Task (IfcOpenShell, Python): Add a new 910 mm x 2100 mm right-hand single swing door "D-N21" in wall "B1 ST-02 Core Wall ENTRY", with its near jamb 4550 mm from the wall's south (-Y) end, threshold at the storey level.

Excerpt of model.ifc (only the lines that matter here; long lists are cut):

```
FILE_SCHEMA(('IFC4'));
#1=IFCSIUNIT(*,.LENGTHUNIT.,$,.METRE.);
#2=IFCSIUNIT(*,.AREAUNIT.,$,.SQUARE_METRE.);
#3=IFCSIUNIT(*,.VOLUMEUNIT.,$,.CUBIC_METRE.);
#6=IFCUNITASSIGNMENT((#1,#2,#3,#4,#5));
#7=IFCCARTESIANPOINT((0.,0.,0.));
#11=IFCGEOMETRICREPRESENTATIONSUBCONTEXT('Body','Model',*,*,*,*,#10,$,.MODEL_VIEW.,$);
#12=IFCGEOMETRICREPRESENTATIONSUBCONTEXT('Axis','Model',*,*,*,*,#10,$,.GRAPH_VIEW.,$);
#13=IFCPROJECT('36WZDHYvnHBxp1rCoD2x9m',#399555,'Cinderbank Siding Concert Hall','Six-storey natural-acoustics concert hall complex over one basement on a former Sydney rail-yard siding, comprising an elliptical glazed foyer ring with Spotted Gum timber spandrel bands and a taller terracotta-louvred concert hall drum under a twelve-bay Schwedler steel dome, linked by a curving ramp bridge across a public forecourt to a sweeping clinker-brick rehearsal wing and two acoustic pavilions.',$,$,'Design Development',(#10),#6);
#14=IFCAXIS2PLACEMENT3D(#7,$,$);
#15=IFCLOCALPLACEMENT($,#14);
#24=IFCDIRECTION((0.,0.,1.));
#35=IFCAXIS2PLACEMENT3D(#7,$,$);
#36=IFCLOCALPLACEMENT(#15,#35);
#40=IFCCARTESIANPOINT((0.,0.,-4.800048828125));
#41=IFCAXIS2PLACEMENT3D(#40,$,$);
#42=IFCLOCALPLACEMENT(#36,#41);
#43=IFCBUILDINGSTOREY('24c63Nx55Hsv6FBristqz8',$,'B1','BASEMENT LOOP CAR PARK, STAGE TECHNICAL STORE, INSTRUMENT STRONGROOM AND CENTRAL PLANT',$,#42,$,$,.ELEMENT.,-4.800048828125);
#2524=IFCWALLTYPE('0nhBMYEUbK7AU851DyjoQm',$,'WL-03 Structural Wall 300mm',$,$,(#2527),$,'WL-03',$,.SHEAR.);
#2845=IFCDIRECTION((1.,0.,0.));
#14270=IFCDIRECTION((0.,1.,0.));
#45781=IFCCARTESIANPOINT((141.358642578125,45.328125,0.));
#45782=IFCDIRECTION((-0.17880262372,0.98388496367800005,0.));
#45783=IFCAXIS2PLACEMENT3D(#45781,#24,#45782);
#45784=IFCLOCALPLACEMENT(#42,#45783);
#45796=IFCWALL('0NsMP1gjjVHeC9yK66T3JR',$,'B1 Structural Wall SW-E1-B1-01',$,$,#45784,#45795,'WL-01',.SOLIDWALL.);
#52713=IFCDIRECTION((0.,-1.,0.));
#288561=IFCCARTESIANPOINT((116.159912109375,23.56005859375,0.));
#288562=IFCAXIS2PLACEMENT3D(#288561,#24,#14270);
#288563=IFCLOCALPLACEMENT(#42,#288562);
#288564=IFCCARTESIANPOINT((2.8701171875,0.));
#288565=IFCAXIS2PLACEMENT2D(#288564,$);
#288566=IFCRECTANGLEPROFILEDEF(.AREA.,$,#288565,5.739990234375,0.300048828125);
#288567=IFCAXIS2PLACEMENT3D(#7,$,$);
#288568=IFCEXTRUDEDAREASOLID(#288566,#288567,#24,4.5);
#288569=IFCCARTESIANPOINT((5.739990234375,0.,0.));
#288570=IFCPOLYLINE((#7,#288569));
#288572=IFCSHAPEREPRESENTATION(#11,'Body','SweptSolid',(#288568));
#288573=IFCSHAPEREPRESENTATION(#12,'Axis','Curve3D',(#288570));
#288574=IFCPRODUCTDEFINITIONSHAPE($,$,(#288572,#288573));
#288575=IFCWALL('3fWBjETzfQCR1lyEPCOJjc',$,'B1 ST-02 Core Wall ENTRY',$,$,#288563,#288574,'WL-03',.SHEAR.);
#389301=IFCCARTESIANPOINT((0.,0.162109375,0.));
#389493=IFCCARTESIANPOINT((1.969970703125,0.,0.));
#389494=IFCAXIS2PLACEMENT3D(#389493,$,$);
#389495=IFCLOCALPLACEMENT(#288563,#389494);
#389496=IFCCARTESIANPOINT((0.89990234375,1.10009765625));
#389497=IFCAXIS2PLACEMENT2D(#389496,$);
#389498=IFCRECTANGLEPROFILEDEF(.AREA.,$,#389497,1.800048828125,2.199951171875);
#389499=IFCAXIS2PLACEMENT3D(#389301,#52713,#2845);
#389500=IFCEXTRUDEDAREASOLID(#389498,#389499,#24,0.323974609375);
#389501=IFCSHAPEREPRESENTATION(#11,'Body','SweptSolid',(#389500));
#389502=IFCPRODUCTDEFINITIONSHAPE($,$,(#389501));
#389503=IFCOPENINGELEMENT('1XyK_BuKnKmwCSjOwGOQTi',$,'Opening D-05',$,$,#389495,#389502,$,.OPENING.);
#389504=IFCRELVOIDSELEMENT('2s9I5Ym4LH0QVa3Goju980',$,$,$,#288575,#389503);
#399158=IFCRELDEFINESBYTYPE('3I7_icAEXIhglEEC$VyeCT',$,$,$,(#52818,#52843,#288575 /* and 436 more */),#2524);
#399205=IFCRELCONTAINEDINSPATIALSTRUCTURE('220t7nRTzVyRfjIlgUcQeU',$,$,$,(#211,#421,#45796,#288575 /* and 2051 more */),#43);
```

```python
import numpy as np
import ifcopenshell
import ifcopenshell.api.feature
import ifcopenshell.api.geometry
import ifcopenshell.api.root
import ifcopenshell.api.spatial
import ifcopenshell.geom
import ifcopenshell.util.element
import ifcopenshell.util.placement
import ifcopenshell.util.representation
import ifcopenshell.util.shape
import ifcopenshell.util.unit

model = ifcopenshell.open("model.ifc")
unit_scale = ifcopenshell.util.unit.calculate_unit_scale(model)
settings = ifcopenshell.geom.settings()


def volume(element):
    """Net volume in cubic metres, openings subtracted."""
    shape = ifcopenshell.geom.create_shape(settings, element)
    return ifcopenshell.util.shape.get_volume(shape.geometry)


wall = model.by_guid("3fWBjETzfQCR1lyEPCOJjc")
storey = ifcopenshell.util.element.get_container(wall, ifc_class="IfcBuildingStorey")
context = ifcopenshell.util.representation.get_context(model, "Model", "Body", "MODEL_VIEW")
before = volume(wall)

width, height, from_end, sill = 0.91, 2.1, 4.55, 0.0  # metres

# The wall runs along its own X axis, and the end named is its -X end.
wall_shape = ifcopenshell.geom.create_shape(settings, wall)
x, y, z = ifcopenshell.util.shape.get_vertices(wall_shape.geometry).T
start = x.min() + from_end
face, thickness = float(y.min()), float(y.max() - y.min())
wall_matrix = ifcopenshell.util.placement.get_local_placement(wall.ObjectPlacement)
level = ifcopenshell.util.placement.get_local_placement(storey.ObjectPlacement)[2, 3]


def in_wall(x, y):
    """Placement at x, y metres in the wall's axes, at sill height."""
    matrix = wall_matrix.copy()
    matrix[:, 3] = wall_matrix @ np.array([x / unit_scale, y / unit_scale, 0.0, 1.0])
    matrix[2, 3] = level + sill / unit_scale
    return matrix


# Opening: a box that overshoots both wall faces by 50 mm.
opening = ifcopenshell.api.root.create_entity(model, ifc_class="IfcOpeningElement", predefined_type="OPENING")
box = ifcopenshell.api.geometry.add_wall_representation(
    model, context=context, length=width, height=height, thickness=thickness + 0.1
)
ifcopenshell.api.geometry.assign_representation(model, product=opening, representation=box)
ifcopenshell.api.geometry.edit_object_placement(model, product=opening, matrix=in_wall(start, face - 0.05), is_si=False)
ifcopenshell.api.feature.add_feature(model, feature=opening, element=wall)

door = ifcopenshell.api.root.create_entity(model, ifc_class="IfcDoor", name="D-N21", predefined_type="DOOR")
door.OverallWidth, door.OverallHeight = width / unit_scale, height / unit_scale
door.OperationType = "SINGLE_SWING_RIGHT"
body = ifcopenshell.api.geometry.add_door_representation(
    model,
    context=context,
    overall_width=door.OverallWidth,
    overall_height=door.OverallHeight,
    operation_type="SINGLE_SWING_RIGHT",
    lining_properties={"LiningDepth": thickness / unit_scale, "ThresholdDepth": thickness / unit_scale},
)
ifcopenshell.api.geometry.assign_representation(model, product=door, representation=body)
ifcopenshell.api.spatial.assign_container(model, products=[door], relating_structure=storey)
ifcopenshell.api.feature.add_filling(model, opening=opening, element=door)

# The lining spans the wall, so the door starts at the wall face.
ifcopenshell.api.geometry.edit_object_placement(model, product=door, matrix=in_wall(start, face), is_si=False)

after = volume(wall)

print(f"wall volume {before:.3f} -> {after:.3f} m3")

model.write("model_edited.ifc")
```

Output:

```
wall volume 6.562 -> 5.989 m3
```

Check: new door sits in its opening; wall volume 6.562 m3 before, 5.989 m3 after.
